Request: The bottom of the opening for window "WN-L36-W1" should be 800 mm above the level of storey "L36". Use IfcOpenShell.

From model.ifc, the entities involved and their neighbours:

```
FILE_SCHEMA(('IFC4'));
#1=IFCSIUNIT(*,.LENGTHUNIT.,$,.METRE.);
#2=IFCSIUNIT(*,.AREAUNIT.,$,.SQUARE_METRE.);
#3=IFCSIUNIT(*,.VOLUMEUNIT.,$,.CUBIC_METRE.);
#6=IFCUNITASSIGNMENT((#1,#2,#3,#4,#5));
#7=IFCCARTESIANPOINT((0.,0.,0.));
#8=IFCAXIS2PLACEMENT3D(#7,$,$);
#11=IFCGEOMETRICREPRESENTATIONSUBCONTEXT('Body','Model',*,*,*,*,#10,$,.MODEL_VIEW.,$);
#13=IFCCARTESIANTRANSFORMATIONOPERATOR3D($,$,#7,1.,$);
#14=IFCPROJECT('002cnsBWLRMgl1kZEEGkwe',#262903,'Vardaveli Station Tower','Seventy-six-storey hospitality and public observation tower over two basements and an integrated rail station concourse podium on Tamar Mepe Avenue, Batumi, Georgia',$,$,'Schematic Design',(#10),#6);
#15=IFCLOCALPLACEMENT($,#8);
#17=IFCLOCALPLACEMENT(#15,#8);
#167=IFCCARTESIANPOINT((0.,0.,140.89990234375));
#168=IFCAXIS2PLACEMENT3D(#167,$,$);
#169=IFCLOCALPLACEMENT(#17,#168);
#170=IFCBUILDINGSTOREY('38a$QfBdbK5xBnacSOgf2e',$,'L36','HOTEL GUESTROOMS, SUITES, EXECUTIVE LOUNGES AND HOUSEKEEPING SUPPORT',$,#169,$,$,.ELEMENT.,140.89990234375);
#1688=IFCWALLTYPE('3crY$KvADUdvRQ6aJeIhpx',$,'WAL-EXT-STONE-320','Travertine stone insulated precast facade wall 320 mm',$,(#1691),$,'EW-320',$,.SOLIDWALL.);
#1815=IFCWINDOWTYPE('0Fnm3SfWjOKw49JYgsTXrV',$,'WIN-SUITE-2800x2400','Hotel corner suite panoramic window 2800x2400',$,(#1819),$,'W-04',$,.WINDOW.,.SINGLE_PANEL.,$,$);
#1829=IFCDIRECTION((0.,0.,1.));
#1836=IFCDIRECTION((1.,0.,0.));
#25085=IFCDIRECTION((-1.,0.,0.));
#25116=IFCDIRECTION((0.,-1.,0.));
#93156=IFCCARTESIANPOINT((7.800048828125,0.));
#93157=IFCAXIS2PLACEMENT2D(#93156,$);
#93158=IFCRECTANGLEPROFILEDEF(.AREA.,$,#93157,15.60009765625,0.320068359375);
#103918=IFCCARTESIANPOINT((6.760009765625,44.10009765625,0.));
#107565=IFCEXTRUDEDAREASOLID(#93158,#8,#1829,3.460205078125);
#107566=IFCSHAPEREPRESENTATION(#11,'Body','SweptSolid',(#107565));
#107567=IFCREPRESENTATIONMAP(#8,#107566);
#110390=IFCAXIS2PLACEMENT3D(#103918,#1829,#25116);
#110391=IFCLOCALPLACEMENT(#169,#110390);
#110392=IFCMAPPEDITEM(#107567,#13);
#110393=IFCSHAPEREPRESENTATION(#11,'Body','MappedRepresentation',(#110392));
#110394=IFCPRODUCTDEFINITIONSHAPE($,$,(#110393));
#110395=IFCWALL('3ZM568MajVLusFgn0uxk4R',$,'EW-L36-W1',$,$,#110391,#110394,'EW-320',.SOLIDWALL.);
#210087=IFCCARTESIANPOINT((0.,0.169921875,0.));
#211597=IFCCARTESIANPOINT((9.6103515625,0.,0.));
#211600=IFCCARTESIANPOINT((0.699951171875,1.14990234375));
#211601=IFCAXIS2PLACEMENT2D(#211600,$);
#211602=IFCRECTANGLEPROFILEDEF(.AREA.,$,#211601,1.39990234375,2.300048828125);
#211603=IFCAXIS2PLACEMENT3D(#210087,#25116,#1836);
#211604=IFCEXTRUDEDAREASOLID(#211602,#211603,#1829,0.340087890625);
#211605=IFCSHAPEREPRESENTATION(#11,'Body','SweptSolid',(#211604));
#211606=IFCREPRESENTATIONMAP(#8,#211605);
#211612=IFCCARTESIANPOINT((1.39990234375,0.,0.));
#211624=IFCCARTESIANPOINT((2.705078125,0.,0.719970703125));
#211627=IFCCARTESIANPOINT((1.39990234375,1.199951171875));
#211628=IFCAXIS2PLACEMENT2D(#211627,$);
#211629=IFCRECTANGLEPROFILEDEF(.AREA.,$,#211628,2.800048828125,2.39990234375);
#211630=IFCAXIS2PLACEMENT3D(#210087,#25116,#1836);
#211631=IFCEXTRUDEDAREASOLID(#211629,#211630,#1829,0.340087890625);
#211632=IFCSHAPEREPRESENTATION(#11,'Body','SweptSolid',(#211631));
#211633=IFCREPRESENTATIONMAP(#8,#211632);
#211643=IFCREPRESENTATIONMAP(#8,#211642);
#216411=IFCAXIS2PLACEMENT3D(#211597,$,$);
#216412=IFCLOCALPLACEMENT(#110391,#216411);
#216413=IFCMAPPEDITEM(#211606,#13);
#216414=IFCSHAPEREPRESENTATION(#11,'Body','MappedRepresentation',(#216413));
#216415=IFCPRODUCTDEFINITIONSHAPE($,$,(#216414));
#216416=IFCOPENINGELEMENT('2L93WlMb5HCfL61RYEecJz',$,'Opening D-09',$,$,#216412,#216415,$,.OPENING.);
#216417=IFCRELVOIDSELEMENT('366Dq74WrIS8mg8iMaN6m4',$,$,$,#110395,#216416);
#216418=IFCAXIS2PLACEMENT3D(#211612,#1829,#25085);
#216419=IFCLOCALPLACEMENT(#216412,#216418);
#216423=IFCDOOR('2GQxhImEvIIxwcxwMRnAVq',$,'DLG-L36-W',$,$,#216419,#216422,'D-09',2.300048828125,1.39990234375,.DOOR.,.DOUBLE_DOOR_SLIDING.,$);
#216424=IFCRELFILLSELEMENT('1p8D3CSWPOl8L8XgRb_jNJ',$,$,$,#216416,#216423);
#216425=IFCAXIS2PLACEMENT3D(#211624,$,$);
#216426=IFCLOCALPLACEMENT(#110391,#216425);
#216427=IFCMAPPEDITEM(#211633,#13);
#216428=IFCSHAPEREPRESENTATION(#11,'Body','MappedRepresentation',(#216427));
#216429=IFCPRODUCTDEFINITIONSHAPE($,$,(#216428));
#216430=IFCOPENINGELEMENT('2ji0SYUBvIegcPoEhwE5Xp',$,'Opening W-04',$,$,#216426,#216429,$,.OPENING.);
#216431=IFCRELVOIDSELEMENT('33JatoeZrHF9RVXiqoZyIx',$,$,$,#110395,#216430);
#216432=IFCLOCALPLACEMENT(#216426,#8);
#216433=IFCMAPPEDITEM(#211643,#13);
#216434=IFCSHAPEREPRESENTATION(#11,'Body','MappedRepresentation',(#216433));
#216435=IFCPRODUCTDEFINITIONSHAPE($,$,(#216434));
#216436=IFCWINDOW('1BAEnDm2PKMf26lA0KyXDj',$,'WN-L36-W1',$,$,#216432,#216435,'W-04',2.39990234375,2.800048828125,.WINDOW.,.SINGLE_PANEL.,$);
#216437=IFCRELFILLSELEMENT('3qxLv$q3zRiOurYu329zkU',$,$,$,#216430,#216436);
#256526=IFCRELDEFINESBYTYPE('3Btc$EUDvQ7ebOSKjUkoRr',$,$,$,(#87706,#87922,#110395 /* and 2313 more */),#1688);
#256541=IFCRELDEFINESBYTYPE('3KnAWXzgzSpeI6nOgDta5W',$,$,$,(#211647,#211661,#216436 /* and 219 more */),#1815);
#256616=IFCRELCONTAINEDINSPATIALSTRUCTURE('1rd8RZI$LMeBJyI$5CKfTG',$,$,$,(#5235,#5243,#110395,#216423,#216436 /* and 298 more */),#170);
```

```python
import numpy as np
import ifcopenshell
import ifcopenshell.api.geometry
import ifcopenshell.geom
import ifcopenshell.util.element
import ifcopenshell.util.placement
import ifcopenshell.util.shape
import ifcopenshell.util.unit

model = ifcopenshell.open("model.ifc")
unit_scale = ifcopenshell.util.unit.calculate_unit_scale(model)

window = model.by_id(216436)
opening = window.FillsVoids[0].RelatingOpeningElement
storey = ifcopenshell.util.element.get_container(window, ifc_class="IfcBuildingStorey")
level = ifcopenshell.util.placement.get_local_placement(storey.ObjectPlacement)[2, 3]

# The opening's origin need not be at the sill, so measure its lowest point.
shape = ifcopenshell.geom.create_shape(ifcopenshell.geom.settings(), opening)
bottom = ifcopenshell.util.shape.get_shape_bottom_elevation(shape, shape.geometry) / unit_scale
dz = level + 0.8 / unit_scale - bottom

shift = np.array([0.0, 0.0, dz])
# The window is placed relative to its opening, so it follows when the opening moves.
matrix = ifcopenshell.util.placement.get_local_placement(opening.ObjectPlacement)
matrix[:3, 3] += shift
ifcopenshell.api.geometry.edit_object_placement(
    model, product=opening, matrix=matrix, is_si=False, should_transform_children=True
)

print(f"moved by {dz * unit_scale:+.3f} m")

model.write("model_v2.ifc")
```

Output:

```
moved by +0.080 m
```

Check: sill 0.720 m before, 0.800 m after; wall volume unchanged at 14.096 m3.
